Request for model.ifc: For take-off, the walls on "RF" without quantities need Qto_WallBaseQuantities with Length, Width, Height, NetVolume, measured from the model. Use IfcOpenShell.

First a look at what the model holds.

```python
import ifcopenshell
import ifcopenshell.util.element
import ifcopenshell.util.unit

model = ifcopenshell.open("model.ifc")
print(model.schema)
for unit_type in ("LENGTHUNIT", "AREAUNIT", "VOLUMEUNIT"):
    print(unit_type, ifcopenshell.util.unit.calculate_unit_scale(model, unit_type))
storey = next(s for s in model.by_type("IfcBuildingStorey") if s.Name == "RF")
walls = [e for e in ifcopenshell.util.element.get_decomposition(storey) if e.is_a("IfcWall")]
for e in sorted(walls, key=lambda e: e.id()):
    print(e.id(), e.is_a(), e.Name, list(ifcopenshell.util.element.get_psets(e, qtos_only=True)), sep=" | ")
```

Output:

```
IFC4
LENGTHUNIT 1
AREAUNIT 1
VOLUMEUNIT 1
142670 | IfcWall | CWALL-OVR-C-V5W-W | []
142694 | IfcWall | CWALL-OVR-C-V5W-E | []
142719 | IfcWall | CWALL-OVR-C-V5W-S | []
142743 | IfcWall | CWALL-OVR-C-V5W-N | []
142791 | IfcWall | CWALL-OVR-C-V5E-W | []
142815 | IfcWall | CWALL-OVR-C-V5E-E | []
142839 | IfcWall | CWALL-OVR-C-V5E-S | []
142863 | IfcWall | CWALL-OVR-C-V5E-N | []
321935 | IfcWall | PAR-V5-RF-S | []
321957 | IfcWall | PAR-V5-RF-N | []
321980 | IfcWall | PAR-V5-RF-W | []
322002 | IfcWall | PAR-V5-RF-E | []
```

```python
import ifcopenshell
import ifcopenshell.api.pset
import ifcopenshell.geom
import ifcopenshell.util.element
import ifcopenshell.util.shape
import ifcopenshell.util.unit

model = ifcopenshell.open("model.ifc")
unit_scale = ifcopenshell.util.unit.calculate_unit_scale(model)
volume_scale = ifcopenshell.util.unit.calculate_unit_scale(model, "VOLUMEUNIT")
settings = ifcopenshell.geom.settings()

storey = next(s for s in model.by_type("IfcBuildingStorey") if s.Name == "RF")
walls = [e for e in ifcopenshell.util.element.get_decomposition(storey) if e.is_a("IfcWall")]

for e in sorted(walls, key=lambda e: e.id()):
    if ifcopenshell.util.element.get_psets(e, qtos_only=True, should_inherit=False):
        continue
    # Geometry comes back in metres, in the element's own axes.
    shape = ifcopenshell.geom.create_shape(settings, e)
    values = {
        "Length": ifcopenshell.util.shape.get_x(shape.geometry) / unit_scale,
        "Width": ifcopenshell.util.shape.get_y(shape.geometry) / unit_scale,
        "Height": ifcopenshell.util.shape.get_z(shape.geometry) / unit_scale,
        "NetVolume": ifcopenshell.util.shape.get_volume(shape.geometry) / volume_scale,
    }
    qto = ifcopenshell.api.pset.add_qto(model, product=e, name="Qto_WallBaseQuantities")
    ifcopenshell.api.pset.edit_qto(model, qto=qto, properties=values)
    print(e.id(), {k: round(v, 3) for k, v in values.items()})

model.write("model_v2.ifc")
```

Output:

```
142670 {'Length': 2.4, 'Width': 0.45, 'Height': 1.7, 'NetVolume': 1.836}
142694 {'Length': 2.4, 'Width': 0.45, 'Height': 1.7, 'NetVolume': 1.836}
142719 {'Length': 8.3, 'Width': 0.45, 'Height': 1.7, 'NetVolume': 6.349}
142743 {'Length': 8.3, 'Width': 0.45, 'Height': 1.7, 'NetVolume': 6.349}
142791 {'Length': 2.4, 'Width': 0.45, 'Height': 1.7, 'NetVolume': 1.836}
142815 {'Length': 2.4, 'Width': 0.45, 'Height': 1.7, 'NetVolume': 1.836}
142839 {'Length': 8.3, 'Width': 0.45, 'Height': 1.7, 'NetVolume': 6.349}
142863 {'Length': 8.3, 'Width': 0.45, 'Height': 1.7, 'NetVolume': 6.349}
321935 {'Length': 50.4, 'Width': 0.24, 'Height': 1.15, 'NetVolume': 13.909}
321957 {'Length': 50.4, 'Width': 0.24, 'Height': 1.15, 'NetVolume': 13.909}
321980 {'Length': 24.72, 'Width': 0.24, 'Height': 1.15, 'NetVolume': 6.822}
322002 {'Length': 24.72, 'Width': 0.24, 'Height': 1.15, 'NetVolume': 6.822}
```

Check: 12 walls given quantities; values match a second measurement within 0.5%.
